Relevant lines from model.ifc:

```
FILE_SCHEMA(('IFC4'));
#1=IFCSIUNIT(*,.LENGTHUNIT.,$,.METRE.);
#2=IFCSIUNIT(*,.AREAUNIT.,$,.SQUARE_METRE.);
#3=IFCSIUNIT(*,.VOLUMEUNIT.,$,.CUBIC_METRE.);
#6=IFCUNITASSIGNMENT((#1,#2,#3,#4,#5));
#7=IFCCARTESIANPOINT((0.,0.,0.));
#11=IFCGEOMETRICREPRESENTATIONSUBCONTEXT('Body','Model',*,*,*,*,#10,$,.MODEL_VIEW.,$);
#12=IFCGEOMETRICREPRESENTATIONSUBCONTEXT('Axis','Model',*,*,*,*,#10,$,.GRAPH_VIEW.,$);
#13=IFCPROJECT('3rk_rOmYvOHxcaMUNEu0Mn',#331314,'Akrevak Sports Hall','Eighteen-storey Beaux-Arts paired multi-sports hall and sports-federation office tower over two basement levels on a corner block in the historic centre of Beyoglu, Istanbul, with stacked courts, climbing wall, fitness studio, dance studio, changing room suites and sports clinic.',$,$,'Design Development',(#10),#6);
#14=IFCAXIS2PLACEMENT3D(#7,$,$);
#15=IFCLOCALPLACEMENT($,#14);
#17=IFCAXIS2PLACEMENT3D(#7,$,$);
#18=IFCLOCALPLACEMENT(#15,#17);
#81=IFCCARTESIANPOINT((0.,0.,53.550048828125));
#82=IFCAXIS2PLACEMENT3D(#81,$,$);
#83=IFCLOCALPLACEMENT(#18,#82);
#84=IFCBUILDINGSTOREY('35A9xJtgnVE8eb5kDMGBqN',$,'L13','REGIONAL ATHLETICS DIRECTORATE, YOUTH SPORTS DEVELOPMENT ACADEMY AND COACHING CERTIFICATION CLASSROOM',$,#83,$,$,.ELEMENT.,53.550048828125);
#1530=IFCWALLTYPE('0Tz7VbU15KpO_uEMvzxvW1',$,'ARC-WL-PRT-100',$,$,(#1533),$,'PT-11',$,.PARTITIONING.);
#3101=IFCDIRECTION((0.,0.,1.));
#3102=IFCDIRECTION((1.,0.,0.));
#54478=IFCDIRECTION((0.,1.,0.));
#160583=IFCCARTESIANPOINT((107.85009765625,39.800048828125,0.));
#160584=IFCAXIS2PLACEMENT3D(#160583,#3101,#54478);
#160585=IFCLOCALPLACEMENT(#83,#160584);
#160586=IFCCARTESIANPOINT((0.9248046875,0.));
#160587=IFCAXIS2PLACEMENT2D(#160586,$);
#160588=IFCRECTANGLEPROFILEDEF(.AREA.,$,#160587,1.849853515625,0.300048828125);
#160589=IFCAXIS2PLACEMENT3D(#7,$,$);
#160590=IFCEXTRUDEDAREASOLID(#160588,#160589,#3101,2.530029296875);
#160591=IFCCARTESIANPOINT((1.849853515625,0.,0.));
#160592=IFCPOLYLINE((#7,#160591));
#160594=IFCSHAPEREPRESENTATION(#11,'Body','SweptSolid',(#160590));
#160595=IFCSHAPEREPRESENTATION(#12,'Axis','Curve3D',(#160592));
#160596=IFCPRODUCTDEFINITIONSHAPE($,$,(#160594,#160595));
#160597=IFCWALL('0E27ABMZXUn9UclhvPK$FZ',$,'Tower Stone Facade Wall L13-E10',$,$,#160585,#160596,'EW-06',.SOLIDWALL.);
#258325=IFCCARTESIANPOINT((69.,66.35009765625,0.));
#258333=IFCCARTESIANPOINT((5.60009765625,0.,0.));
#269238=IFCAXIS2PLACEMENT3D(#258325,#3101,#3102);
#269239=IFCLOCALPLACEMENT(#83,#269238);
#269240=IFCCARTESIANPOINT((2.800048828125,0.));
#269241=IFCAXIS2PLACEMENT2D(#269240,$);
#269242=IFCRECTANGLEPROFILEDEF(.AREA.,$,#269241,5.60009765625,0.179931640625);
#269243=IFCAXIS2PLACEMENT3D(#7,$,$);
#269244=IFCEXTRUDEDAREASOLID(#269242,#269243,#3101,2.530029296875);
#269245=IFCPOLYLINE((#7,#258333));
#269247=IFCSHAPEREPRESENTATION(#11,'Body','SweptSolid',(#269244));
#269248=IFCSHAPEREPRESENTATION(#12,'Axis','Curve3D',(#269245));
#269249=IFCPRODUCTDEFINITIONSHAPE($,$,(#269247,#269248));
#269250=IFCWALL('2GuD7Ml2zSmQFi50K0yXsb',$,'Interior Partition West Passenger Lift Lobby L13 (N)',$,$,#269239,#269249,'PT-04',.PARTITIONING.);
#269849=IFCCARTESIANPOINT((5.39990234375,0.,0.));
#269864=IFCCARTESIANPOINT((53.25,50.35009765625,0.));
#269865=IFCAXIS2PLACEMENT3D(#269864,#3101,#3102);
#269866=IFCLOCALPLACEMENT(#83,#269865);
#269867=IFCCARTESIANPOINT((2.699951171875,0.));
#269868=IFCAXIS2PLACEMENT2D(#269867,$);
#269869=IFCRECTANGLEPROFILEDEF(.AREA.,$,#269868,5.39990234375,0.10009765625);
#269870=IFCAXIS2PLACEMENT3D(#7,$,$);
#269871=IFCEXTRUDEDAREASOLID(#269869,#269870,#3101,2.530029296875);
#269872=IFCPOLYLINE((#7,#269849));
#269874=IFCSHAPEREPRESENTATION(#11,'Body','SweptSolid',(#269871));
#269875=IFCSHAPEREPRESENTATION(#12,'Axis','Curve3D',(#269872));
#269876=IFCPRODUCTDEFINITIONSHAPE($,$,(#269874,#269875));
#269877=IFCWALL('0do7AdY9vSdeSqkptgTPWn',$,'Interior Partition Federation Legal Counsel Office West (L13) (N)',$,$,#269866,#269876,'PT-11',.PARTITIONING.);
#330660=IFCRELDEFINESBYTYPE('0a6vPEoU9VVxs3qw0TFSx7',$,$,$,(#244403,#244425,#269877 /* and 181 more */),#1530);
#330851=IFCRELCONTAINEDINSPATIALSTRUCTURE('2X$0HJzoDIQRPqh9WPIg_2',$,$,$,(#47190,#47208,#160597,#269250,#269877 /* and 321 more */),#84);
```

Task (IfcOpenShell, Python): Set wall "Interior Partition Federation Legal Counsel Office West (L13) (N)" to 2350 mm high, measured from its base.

```python
import ifcopenshell
import ifcopenshell.geom
import ifcopenshell.util.representation
import ifcopenshell.util.shape
import ifcopenshell.util.unit

model = ifcopenshell.open("model.ifc")
unit_scale = ifcopenshell.util.unit.calculate_unit_scale(model)
settings = ifcopenshell.geom.settings()


def volume(element):
    """Net volume in cubic metres, openings subtracted."""
    shape = ifcopenshell.geom.create_shape(settings, element)
    return ifcopenshell.util.shape.get_volume(shape.geometry)


wall = model.by_id(269877)
before = volume(wall)

body = ifcopenshell.util.representation.get_representation(wall, "Model", "Body")
solid = body.Items[0]
old_height = solid.Depth
solid.Depth = 2.35 / unit_scale
after = volume(wall)

print(f"height {old_height:g} -> {solid.Depth:g}, volume {before:.3f} -> {after:.3f} m3")

model.write("model_rev.ifc")
```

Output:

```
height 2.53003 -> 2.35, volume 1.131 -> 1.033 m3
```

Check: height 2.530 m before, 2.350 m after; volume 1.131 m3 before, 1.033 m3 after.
